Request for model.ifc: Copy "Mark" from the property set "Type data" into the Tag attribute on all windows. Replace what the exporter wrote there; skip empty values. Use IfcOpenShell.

First a look at what the model holds.

```python
import ifcopenshell
import ifcopenshell.util.element

model = ifcopenshell.open("model.ifc")
print(model.schema)
windows = model.by_type("IfcWindow")
print(len(windows), "windows")
for e in windows[:8]:
    source = ifcopenshell.util.element.get_pset(e, "Type data", "Mark")
    target = e.Tag
    print(e.id(), repr(source), repr(target), sep=" | ")
```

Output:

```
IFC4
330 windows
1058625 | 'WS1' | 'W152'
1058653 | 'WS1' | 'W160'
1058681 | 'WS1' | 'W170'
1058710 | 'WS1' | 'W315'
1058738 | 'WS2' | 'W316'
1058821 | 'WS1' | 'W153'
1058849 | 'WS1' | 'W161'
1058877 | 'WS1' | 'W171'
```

```python
import ifcopenshell
import ifcopenshell.util.element

model = ifcopenshell.open("model.ifc")

count = 0
for e in model.by_type("IfcWindow"):
    value = ifcopenshell.util.element.get_pset(e, "Type data", "Mark")
    current = e.Tag
    if not value or not value.strip() or current == value:
        continue
    e.Tag = value
    count += 1

print(count, "windows updated")

model.write("model_v2.ifc")
```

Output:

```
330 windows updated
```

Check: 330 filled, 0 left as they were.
